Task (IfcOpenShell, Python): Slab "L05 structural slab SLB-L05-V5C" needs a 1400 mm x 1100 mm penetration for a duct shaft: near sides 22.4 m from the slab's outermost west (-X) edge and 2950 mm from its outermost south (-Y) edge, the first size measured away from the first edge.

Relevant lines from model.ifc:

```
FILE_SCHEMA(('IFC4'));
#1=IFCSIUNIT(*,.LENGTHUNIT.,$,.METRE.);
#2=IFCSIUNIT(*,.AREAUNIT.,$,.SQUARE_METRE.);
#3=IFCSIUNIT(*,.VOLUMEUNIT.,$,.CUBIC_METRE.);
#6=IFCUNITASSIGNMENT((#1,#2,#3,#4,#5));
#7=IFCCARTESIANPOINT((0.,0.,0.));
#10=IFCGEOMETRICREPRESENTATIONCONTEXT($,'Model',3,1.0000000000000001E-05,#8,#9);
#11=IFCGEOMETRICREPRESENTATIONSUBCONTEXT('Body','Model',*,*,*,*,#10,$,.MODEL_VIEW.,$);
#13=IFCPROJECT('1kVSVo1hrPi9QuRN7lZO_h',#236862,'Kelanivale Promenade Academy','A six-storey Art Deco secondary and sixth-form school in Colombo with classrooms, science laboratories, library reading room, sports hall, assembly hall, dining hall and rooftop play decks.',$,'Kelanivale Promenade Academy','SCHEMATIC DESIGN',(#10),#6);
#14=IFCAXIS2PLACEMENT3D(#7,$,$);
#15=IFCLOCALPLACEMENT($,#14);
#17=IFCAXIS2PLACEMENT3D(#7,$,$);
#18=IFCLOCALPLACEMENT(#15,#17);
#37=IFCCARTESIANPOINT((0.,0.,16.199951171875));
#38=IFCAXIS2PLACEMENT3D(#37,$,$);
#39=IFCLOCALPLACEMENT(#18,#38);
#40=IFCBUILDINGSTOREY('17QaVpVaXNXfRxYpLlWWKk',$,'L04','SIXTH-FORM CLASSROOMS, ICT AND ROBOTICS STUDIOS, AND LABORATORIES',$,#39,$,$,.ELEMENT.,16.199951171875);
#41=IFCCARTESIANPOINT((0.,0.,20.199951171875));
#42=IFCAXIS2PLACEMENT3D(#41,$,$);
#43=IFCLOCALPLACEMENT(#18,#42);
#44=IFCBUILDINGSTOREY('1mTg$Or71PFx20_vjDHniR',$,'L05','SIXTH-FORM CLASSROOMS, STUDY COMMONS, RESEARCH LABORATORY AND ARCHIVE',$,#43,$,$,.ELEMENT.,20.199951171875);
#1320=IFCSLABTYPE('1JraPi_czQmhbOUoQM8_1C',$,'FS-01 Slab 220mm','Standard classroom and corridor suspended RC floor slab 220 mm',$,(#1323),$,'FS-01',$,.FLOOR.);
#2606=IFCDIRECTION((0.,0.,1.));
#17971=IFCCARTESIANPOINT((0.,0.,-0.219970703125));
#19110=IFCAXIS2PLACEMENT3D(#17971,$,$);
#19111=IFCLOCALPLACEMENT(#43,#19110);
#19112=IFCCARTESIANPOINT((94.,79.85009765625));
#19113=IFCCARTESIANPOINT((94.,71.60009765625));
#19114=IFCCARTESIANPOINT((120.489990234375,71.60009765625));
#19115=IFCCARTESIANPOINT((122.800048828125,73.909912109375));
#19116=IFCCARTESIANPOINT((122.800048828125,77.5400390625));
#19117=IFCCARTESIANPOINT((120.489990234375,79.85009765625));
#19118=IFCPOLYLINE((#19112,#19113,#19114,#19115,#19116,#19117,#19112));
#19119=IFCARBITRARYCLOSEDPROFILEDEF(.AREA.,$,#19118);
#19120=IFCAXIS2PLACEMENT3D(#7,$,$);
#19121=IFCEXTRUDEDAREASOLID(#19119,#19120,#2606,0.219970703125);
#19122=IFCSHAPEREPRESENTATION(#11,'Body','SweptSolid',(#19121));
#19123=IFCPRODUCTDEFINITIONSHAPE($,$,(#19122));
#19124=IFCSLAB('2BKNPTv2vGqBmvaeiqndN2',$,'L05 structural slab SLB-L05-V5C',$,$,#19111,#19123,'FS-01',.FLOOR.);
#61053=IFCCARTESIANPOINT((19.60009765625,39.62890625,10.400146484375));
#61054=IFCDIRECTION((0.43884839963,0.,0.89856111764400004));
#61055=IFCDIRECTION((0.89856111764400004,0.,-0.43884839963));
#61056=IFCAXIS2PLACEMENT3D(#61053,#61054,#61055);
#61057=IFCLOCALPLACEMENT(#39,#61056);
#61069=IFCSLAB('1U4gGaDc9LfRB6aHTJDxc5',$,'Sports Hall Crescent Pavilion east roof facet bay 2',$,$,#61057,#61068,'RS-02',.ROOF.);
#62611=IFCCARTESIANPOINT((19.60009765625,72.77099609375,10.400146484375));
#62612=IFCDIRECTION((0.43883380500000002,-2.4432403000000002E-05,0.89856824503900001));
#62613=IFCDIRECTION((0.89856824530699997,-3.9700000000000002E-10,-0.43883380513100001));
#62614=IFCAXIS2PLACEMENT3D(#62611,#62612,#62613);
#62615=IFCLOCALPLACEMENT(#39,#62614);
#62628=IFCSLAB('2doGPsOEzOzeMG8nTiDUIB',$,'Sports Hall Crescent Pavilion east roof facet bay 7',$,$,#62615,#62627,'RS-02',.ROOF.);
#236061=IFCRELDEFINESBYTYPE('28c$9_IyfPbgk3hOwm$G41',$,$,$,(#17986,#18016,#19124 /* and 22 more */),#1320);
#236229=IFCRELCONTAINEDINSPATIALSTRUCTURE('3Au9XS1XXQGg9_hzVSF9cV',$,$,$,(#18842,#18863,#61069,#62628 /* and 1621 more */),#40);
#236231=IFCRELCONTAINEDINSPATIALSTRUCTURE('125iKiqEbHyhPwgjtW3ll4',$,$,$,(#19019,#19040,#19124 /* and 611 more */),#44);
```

```python
import numpy as np
import ifcopenshell
import ifcopenshell.api.feature
import ifcopenshell.api.geometry
import ifcopenshell.api.root
import ifcopenshell.geom
import ifcopenshell.util.placement
import ifcopenshell.util.representation
import ifcopenshell.util.shape
import ifcopenshell.util.unit

model = ifcopenshell.open("model.ifc")
unit_scale = ifcopenshell.util.unit.calculate_unit_scale(model)
settings = ifcopenshell.geom.settings()


def volume(element):
    """Net volume in cubic metres, openings subtracted."""
    shape = ifcopenshell.geom.create_shape(settings, element)
    return ifcopenshell.util.shape.get_volume(shape.geometry)


slab = model.by_guid("2BKNPTv2vGqBmvaeiqndN2")
before = volume(slab)

# Extent in the slab's own axes, in metres. The edges named are its -X and -Y sides.
slab_shape = ifcopenshell.geom.create_shape(settings, slab)
vertices = ifcopenshell.util.shape.get_vertices(slab_shape.geometry)
x_min, y_min, bottom = vertices.min(axis=0)
top = vertices[:, 2].max()

opening = ifcopenshell.api.root.create_entity(model, ifc_class="IfcOpeningElement", name="Duct shaft opening", predefined_type="OPENING")
context = ifcopenshell.util.representation.get_context(model, "Model", "Body", "MODEL_VIEW")
width, depth = 1.4, 1.1
outline = [(0.0, 0.0), (width, 0.0), (width, depth), (0.0, depth), (0.0, 0.0)]
# Overshoot both faces by 50 mm so the cut is clean.
shape = ifcopenshell.api.geometry.add_slab_representation(
    model, context=context, depth=top - bottom + 0.1, polyline=outline
)
ifcopenshell.api.geometry.assign_representation(model, product=opening, representation=shape)

matrix = ifcopenshell.util.placement.get_local_placement(slab.ObjectPlacement)
matrix[:, 3] = matrix @ np.append(np.array([x_min + 22.4, y_min + 2.95, bottom - 0.05]) / unit_scale, 1.0)
ifcopenshell.api.geometry.edit_object_placement(model, product=opening, matrix=matrix, is_si=False)
ifcopenshell.api.feature.add_feature(model, feature=opening, element=slab)

after = volume(slab)

print(f"slab volume {before:.3f} -> {after:.3f} m3")

model.write("model_updated.ifc")
```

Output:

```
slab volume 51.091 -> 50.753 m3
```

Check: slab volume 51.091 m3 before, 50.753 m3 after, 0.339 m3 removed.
